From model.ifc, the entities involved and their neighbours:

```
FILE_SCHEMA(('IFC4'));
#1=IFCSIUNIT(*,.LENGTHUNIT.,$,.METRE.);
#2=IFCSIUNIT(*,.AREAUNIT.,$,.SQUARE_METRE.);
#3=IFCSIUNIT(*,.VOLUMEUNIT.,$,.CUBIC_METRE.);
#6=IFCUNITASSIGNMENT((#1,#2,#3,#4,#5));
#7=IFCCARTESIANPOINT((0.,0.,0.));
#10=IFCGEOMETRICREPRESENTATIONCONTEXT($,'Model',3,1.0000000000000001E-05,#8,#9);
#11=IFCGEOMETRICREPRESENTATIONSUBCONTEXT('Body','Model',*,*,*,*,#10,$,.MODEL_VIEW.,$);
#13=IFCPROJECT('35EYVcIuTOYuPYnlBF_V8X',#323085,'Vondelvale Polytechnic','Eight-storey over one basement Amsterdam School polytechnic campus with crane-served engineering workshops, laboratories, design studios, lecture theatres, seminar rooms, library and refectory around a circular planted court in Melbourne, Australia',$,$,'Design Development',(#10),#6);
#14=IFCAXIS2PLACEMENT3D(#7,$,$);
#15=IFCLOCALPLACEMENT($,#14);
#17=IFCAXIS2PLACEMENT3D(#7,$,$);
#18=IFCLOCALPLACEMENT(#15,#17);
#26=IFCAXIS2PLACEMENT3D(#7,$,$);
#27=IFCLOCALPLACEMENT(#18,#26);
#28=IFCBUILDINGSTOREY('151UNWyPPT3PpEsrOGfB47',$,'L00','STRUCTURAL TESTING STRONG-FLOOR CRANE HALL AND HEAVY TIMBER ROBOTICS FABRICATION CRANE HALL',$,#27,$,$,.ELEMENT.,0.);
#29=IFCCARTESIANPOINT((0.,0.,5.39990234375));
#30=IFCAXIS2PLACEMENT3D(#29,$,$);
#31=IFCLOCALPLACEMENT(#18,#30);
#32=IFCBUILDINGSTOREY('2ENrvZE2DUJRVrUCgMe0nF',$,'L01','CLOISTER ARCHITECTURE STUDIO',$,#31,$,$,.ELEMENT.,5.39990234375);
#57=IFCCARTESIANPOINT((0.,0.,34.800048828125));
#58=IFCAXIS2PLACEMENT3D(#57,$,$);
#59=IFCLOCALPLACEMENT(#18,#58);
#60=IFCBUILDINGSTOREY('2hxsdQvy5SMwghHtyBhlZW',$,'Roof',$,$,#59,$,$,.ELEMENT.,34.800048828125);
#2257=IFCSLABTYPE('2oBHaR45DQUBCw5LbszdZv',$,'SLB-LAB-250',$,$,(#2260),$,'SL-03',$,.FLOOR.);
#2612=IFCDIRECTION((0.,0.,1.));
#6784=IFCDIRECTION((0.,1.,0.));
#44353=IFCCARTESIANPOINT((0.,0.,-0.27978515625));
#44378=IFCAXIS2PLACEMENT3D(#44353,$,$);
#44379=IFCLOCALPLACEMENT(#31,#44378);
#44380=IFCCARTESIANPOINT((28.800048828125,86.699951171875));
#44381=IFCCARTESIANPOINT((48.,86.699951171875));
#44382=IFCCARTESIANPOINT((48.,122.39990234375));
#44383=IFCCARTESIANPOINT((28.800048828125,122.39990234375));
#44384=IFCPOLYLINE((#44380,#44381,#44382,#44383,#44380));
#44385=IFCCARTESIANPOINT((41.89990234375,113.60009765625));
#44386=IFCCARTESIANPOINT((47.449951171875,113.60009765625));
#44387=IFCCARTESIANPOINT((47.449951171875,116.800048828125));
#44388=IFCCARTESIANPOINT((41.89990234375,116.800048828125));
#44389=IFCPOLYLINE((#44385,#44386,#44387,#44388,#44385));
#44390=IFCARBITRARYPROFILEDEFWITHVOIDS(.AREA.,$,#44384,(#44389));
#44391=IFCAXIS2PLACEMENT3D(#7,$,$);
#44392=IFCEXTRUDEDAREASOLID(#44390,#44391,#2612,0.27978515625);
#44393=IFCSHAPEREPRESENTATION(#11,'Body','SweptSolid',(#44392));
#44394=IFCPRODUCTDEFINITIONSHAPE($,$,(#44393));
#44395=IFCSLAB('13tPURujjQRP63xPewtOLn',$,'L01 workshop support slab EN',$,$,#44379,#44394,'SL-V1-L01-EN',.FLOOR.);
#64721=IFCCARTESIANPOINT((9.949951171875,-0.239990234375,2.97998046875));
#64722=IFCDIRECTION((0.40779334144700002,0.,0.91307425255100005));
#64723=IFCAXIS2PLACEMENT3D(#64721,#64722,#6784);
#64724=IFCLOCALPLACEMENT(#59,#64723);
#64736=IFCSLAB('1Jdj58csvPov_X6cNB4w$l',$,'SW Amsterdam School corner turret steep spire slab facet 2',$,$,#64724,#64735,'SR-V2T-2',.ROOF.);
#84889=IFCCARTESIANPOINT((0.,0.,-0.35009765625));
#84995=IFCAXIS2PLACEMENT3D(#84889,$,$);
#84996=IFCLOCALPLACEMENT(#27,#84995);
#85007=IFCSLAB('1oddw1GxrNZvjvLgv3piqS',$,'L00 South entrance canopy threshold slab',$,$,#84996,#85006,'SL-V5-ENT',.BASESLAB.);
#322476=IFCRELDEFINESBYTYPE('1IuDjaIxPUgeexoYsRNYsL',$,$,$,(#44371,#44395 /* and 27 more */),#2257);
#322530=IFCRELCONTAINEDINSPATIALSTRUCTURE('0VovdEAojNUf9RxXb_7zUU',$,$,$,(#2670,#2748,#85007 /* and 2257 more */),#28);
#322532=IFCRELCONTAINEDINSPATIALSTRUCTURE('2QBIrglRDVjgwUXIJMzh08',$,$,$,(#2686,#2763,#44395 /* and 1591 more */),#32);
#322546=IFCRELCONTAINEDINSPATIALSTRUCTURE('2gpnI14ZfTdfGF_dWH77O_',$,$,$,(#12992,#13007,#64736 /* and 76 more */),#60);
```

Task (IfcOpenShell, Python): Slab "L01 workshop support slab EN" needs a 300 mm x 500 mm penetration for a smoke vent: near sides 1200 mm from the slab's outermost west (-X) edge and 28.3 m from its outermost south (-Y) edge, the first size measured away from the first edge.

```python
import numpy as np
import ifcopenshell
import ifcopenshell.api.feature
import ifcopenshell.api.geometry
import ifcopenshell.api.root
import ifcopenshell.geom
import ifcopenshell.util.placement
import ifcopenshell.util.representation
import ifcopenshell.util.shape
import ifcopenshell.util.unit

model = ifcopenshell.open("model.ifc")
unit_scale = ifcopenshell.util.unit.calculate_unit_scale(model)
settings = ifcopenshell.geom.settings()


def volume(element):
    """Net volume in cubic metres, openings subtracted."""
    shape = ifcopenshell.geom.create_shape(settings, element)
    return ifcopenshell.util.shape.get_volume(shape.geometry)


slab = model.by_guid("13tPURujjQRP63xPewtOLn")
before = volume(slab)

# Extent in the slab's own axes, in metres. The edges named are its -X and -Y sides.
slab_shape = ifcopenshell.geom.create_shape(settings, slab)
vertices = ifcopenshell.util.shape.get_vertices(slab_shape.geometry)
x_min, y_min, bottom = vertices.min(axis=0)
top = vertices[:, 2].max()

opening = ifcopenshell.api.root.create_entity(model, ifc_class="IfcOpeningElement", name="Smoke vent opening", predefined_type="OPENING")
context = ifcopenshell.util.representation.get_context(model, "Model", "Body", "MODEL_VIEW")
width, depth = 0.3, 0.5
outline = [(0.0, 0.0), (width, 0.0), (width, depth), (0.0, depth), (0.0, 0.0)]
# Overshoot both faces by 50 mm so the cut is clean.
shape = ifcopenshell.api.geometry.add_slab_representation(
    model, context=context, depth=top - bottom + 0.1, polyline=outline
)
ifcopenshell.api.geometry.assign_representation(model, product=opening, representation=shape)

matrix = ifcopenshell.util.placement.get_local_placement(slab.ObjectPlacement)
matrix[:, 3] = matrix @ np.append(np.array([x_min + 1.2, y_min + 28.3, bottom - 0.05]) / unit_scale, 1.0)
ifcopenshell.api.geometry.edit_object_placement(model, product=opening, matrix=matrix, is_si=False)
ifcopenshell.api.feature.add_feature(model, feature=opening, element=slab)

after = volume(slab)

print(f"slab volume {before:.3f} -> {after:.3f} m3")

model.write("model-out.ifc")
```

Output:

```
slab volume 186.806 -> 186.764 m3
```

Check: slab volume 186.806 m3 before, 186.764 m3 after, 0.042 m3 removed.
